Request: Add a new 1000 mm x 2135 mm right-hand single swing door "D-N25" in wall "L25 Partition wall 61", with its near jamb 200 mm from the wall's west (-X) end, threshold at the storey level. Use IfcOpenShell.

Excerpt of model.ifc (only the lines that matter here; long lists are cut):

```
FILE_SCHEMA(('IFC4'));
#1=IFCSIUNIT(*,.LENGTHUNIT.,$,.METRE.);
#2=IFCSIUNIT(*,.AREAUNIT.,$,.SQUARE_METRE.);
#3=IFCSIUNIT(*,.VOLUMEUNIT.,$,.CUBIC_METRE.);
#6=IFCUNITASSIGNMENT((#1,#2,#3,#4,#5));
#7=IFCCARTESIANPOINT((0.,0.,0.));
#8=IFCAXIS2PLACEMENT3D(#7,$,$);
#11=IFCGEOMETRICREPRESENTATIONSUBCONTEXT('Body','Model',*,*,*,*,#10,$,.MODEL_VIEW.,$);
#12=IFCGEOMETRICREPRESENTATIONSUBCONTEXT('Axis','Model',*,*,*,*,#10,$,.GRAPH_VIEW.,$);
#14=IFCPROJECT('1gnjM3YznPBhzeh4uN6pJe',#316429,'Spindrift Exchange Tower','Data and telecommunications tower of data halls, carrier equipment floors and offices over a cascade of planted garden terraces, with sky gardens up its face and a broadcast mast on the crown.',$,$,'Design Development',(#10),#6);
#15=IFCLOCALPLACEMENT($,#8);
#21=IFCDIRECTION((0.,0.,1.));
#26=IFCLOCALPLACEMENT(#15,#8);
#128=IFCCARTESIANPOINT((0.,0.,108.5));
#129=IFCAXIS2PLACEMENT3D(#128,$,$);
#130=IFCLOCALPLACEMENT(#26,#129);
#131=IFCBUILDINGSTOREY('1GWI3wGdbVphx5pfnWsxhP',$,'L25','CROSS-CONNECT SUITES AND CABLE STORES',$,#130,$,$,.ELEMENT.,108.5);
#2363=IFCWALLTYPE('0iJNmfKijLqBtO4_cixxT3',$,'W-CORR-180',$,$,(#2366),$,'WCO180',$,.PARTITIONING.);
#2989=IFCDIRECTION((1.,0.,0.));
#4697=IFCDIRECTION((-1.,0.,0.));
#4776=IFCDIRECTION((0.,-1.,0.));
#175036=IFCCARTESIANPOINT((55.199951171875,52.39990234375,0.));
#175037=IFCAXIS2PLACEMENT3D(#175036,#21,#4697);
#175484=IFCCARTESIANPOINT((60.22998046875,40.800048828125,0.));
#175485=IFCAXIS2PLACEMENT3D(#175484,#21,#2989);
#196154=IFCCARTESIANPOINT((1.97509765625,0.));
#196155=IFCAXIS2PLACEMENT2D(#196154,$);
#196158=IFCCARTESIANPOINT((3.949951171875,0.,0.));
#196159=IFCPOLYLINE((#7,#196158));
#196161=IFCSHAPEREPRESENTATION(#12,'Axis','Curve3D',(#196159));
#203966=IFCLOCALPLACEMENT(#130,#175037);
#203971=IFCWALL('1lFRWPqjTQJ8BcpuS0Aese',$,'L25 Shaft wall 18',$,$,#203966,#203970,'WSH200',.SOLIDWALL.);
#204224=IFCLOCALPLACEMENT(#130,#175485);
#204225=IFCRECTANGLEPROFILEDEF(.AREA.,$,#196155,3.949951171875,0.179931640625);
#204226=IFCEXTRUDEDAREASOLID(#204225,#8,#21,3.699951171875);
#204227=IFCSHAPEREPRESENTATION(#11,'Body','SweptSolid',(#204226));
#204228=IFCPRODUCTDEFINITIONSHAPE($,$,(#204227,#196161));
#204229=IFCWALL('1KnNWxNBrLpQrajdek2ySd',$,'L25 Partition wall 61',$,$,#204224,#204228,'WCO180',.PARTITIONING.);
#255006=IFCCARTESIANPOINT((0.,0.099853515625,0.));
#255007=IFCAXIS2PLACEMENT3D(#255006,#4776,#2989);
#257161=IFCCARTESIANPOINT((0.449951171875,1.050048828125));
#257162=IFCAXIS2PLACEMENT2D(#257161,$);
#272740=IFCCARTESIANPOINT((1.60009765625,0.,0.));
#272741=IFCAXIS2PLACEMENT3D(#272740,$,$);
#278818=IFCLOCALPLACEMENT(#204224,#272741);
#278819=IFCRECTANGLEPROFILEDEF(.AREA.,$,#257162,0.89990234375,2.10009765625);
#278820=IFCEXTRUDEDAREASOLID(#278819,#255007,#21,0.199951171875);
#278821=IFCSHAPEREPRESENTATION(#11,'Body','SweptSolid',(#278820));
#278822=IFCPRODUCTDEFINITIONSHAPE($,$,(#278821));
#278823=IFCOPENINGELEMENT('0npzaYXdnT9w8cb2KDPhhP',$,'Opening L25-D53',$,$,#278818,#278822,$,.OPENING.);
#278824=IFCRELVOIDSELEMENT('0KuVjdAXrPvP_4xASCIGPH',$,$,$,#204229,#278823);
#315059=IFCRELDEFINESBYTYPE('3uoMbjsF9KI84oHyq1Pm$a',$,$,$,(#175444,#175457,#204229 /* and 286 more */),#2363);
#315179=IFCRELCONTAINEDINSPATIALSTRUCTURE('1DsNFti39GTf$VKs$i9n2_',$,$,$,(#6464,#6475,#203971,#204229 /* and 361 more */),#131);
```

```python
import numpy as np
import ifcopenshell
import ifcopenshell.api.feature
import ifcopenshell.api.geometry
import ifcopenshell.api.root
import ifcopenshell.api.spatial
import ifcopenshell.geom
import ifcopenshell.util.element
import ifcopenshell.util.placement
import ifcopenshell.util.representation
import ifcopenshell.util.shape
import ifcopenshell.util.unit

model = ifcopenshell.open("model.ifc")
unit_scale = ifcopenshell.util.unit.calculate_unit_scale(model)
settings = ifcopenshell.geom.settings()


def volume(element):
    """Net volume in cubic metres, openings subtracted."""
    shape = ifcopenshell.geom.create_shape(settings, element)
    return ifcopenshell.util.shape.get_volume(shape.geometry)


wall = model.by_guid("1KnNWxNBrLpQrajdek2ySd")
storey = ifcopenshell.util.element.get_container(wall, ifc_class="IfcBuildingStorey")
context = ifcopenshell.util.representation.get_context(model, "Model", "Body", "MODEL_VIEW")
before = volume(wall)

width, height, from_end, sill = 1, 2.135, 0.2, 0.0  # metres

# The wall runs along its own X axis, and the end named is its -X end.
wall_shape = ifcopenshell.geom.create_shape(settings, wall)
x, y, z = ifcopenshell.util.shape.get_vertices(wall_shape.geometry).T
start = x.min() + from_end
face, thickness = float(y.min()), float(y.max() - y.min())
wall_matrix = ifcopenshell.util.placement.get_local_placement(wall.ObjectPlacement)
level = ifcopenshell.util.placement.get_local_placement(storey.ObjectPlacement)[2, 3]


def in_wall(x, y):
    """Placement at x, y metres in the wall's axes, at sill height."""
    matrix = wall_matrix.copy()
    matrix[:, 3] = wall_matrix @ np.array([x / unit_scale, y / unit_scale, 0.0, 1.0])
    matrix[2, 3] = level + sill / unit_scale
    return matrix


# Opening: a box that overshoots both wall faces by 50 mm.
opening = ifcopenshell.api.root.create_entity(model, ifc_class="IfcOpeningElement", predefined_type="OPENING")
box = ifcopenshell.api.geometry.add_wall_representation(
    model, context=context, length=width, height=height, thickness=thickness + 0.1
)
ifcopenshell.api.geometry.assign_representation(model, product=opening, representation=box)
ifcopenshell.api.geometry.edit_object_placement(model, product=opening, matrix=in_wall(start, face - 0.05), is_si=False)
ifcopenshell.api.feature.add_feature(model, feature=opening, element=wall)

door = ifcopenshell.api.root.create_entity(model, ifc_class="IfcDoor", name="D-N25", predefined_type="DOOR")
door.OverallWidth, door.OverallHeight = width / unit_scale, height / unit_scale
door.OperationType = "SINGLE_SWING_RIGHT"
body = ifcopenshell.api.geometry.add_door_representation(
    model,
    context=context,
    overall_width=door.OverallWidth,
    overall_height=door.OverallHeight,
    operation_type="SINGLE_SWING_RIGHT",
    lining_properties={"LiningDepth": thickness / unit_scale, "ThresholdDepth": thickness / unit_scale},
)
ifcopenshell.api.geometry.assign_representation(model, product=door, representation=body)
ifcopenshell.api.spatial.assign_container(model, products=[door], relating_structure=storey)
ifcopenshell.api.feature.add_filling(model, opening=opening, element=door)

# The lining spans the wall, so the door starts at the wall face.
ifcopenshell.api.geometry.edit_object_placement(model, product=door, matrix=in_wall(start, face), is_si=False)

after = volume(wall)

print(f"wall volume {before:.3f} -> {after:.3f} m3")

model.write("model-out.ifc")
```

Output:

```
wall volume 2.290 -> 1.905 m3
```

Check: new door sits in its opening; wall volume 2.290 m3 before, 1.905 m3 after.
